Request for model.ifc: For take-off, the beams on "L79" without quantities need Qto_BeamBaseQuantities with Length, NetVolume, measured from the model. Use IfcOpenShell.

First a look at what the model holds.

```python
import ifcopenshell
import ifcopenshell.util.element
import ifcopenshell.util.unit

model = ifcopenshell.open("model.ifc")
print(model.schema)
for unit_type in ("LENGTHUNIT", "AREAUNIT", "VOLUMEUNIT"):
    print(unit_type, ifcopenshell.util.unit.calculate_unit_scale(model, unit_type))
storey = next(s for s in model.by_type("IfcBuildingStorey") if s.Name == "L79")
beams = [e for e in ifcopenshell.util.element.get_decomposition(storey) if e.is_a("IfcBeam")]
for e in sorted(beams, key=lambda e: e.id()):
    print(e.id(), e.is_a(), e.Name, list(ifcopenshell.util.element.get_psets(e, qtos_only=True)), sep=" | ")
```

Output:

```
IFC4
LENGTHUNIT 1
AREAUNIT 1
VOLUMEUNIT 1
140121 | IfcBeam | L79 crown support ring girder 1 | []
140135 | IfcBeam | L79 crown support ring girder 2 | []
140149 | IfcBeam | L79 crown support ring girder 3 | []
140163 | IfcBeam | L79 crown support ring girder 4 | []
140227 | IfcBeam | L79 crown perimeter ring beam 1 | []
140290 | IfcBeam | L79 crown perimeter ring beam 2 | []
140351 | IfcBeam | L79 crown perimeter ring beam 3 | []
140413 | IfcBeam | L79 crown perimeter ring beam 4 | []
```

```python
import ifcopenshell
import ifcopenshell.api.pset
import ifcopenshell.geom
import ifcopenshell.util.element
import ifcopenshell.util.shape
import ifcopenshell.util.unit

model = ifcopenshell.open("model.ifc")
unit_scale = ifcopenshell.util.unit.calculate_unit_scale(model)
volume_scale = ifcopenshell.util.unit.calculate_unit_scale(model, "VOLUMEUNIT")
settings = ifcopenshell.geom.settings()

storey = next(s for s in model.by_type("IfcBuildingStorey") if s.Name == "L79")
beams = [e for e in ifcopenshell.util.element.get_decomposition(storey) if e.is_a("IfcBeam")]

for e in sorted(beams, key=lambda e: e.id()):
    if ifcopenshell.util.element.get_psets(e, qtos_only=True, should_inherit=False):
        continue
    # Geometry comes back in metres, in the element's own axes.
    shape = ifcopenshell.geom.create_shape(settings, e)
    values = {
        "Length": ifcopenshell.util.shape.get_max_xyz(shape.geometry) / unit_scale,
        "NetVolume": ifcopenshell.util.shape.get_volume(shape.geometry) / volume_scale,
    }
    qto = ifcopenshell.api.pset.add_qto(model, product=e, name="Qto_BeamBaseQuantities")
    ifcopenshell.api.pset.edit_qto(model, qto=qto, properties=values)
    print(e.id(), {k: round(v, 3) for k, v in values.items()})

model.write("model_updated.ifc")
```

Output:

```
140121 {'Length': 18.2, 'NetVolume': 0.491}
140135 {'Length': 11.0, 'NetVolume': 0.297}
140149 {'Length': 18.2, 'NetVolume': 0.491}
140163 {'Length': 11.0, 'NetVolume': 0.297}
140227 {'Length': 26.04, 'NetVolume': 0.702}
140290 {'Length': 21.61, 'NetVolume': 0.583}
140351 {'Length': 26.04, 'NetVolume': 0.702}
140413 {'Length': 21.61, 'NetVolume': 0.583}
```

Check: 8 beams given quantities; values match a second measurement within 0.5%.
